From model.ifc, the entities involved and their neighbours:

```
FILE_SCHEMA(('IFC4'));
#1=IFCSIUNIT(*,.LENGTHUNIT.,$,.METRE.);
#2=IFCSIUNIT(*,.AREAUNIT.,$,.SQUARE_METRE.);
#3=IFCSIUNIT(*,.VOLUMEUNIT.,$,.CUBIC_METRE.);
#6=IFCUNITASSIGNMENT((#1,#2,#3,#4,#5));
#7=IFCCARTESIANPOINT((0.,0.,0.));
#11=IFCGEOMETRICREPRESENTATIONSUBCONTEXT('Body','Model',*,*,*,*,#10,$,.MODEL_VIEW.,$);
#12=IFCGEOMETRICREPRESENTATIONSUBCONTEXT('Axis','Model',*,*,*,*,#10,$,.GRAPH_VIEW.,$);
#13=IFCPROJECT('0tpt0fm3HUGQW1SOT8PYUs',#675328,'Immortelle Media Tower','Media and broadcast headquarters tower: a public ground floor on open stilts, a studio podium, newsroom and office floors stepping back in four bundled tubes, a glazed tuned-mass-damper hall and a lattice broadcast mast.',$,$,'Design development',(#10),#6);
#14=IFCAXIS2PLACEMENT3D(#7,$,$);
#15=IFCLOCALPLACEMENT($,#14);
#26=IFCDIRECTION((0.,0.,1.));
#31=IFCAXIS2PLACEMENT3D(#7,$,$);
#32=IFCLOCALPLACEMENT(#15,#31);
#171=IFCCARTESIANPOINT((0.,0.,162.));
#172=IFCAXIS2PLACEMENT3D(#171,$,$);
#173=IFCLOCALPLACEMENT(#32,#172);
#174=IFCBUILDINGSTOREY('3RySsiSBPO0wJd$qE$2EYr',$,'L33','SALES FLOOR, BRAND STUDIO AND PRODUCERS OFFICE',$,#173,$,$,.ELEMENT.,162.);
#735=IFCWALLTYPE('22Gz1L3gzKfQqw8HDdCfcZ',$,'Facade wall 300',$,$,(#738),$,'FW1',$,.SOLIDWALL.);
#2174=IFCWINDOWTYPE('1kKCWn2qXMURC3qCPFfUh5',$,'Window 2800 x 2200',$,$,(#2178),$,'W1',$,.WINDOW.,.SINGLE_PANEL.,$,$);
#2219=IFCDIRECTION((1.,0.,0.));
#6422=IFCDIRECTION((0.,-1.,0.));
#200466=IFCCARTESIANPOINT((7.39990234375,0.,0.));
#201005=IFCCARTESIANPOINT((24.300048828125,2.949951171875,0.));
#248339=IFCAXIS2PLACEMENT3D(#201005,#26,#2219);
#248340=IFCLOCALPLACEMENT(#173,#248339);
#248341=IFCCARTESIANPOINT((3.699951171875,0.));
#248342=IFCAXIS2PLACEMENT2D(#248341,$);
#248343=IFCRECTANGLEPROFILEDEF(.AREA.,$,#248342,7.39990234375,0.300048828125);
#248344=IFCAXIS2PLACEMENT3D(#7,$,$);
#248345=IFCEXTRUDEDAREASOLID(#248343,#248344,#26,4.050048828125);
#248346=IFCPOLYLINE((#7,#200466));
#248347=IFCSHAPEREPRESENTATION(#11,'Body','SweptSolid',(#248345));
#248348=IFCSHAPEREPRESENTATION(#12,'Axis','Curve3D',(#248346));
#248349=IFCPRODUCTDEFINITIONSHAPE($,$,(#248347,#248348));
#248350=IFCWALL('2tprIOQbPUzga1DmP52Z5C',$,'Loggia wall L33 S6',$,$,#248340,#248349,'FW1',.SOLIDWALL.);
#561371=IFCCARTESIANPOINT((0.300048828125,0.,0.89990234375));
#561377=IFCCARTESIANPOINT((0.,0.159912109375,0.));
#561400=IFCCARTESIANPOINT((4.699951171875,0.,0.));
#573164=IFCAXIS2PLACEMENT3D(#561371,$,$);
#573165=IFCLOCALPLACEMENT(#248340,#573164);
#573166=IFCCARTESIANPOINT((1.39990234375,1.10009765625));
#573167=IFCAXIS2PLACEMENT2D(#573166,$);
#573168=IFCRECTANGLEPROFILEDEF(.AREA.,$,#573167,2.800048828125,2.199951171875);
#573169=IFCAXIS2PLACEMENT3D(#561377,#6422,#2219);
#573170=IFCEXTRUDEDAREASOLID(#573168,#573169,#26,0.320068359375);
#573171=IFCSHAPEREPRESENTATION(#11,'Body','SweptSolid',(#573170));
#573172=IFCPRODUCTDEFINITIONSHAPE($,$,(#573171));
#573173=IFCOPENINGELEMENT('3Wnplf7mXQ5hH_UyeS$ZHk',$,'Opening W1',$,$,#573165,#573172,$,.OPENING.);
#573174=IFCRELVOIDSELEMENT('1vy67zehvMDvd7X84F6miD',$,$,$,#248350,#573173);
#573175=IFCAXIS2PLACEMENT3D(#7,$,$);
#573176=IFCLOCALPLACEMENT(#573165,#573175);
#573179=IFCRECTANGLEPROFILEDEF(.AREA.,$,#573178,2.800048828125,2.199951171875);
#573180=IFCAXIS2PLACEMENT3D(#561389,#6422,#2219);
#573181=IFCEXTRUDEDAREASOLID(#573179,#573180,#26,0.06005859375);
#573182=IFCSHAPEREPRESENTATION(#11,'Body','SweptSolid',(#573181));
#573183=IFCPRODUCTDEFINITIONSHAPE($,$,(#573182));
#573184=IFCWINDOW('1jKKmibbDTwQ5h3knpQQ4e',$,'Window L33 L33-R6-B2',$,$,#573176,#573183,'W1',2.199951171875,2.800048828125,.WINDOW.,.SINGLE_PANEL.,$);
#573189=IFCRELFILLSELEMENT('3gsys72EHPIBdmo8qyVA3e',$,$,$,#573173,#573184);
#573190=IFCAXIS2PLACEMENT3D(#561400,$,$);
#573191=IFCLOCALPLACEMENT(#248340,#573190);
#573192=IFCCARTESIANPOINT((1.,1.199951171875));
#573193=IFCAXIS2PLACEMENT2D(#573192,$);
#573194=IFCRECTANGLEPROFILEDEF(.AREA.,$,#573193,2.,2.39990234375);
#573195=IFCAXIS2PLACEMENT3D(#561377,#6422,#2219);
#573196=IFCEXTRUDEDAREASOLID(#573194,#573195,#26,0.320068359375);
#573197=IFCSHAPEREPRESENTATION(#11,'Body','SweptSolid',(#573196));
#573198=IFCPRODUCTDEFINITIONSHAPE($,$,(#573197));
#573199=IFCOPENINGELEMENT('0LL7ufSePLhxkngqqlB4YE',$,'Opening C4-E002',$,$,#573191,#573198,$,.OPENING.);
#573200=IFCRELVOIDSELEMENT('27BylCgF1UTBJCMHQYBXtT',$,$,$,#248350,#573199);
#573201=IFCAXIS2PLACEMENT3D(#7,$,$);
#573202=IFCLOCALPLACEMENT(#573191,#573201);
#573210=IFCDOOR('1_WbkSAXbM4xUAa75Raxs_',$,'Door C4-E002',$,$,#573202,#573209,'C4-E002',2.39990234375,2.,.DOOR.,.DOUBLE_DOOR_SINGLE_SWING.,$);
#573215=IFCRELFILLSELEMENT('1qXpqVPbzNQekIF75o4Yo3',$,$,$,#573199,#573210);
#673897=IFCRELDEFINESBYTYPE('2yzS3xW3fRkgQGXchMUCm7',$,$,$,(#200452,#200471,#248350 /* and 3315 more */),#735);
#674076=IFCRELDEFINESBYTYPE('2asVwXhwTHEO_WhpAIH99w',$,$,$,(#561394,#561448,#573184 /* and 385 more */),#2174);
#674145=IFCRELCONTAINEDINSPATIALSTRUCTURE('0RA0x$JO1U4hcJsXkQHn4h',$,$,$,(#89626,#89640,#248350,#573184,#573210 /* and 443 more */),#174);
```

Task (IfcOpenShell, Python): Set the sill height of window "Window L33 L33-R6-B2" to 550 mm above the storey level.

```python
import numpy as np
import ifcopenshell
import ifcopenshell.api.geometry
import ifcopenshell.geom
import ifcopenshell.util.element
import ifcopenshell.util.placement
import ifcopenshell.util.shape
import ifcopenshell.util.unit

model = ifcopenshell.open("model.ifc")
unit_scale = ifcopenshell.util.unit.calculate_unit_scale(model)

window = model.by_id(573184)
opening = window.FillsVoids[0].RelatingOpeningElement
storey = ifcopenshell.util.element.get_container(window, ifc_class="IfcBuildingStorey")
level = ifcopenshell.util.placement.get_local_placement(storey.ObjectPlacement)[2, 3]

# The opening's origin need not be at the sill, so measure its lowest point.
shape = ifcopenshell.geom.create_shape(ifcopenshell.geom.settings(), opening)
bottom = ifcopenshell.util.shape.get_shape_bottom_elevation(shape, shape.geometry) / unit_scale
dz = level + 0.55 / unit_scale - bottom

shift = np.array([0.0, 0.0, dz])
# The window is placed relative to its opening, so it follows when the opening moves.
matrix = ifcopenshell.util.placement.get_local_placement(opening.ObjectPlacement)
matrix[:3, 3] += shift
ifcopenshell.api.geometry.edit_object_placement(
    model, product=opening, matrix=matrix, is_si=False, should_transform_children=True
)

print(f"moved by {dz * unit_scale:+.3f} m")

model.write("model_updated.ifc")
```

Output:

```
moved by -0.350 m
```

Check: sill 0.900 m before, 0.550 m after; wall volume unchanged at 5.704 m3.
